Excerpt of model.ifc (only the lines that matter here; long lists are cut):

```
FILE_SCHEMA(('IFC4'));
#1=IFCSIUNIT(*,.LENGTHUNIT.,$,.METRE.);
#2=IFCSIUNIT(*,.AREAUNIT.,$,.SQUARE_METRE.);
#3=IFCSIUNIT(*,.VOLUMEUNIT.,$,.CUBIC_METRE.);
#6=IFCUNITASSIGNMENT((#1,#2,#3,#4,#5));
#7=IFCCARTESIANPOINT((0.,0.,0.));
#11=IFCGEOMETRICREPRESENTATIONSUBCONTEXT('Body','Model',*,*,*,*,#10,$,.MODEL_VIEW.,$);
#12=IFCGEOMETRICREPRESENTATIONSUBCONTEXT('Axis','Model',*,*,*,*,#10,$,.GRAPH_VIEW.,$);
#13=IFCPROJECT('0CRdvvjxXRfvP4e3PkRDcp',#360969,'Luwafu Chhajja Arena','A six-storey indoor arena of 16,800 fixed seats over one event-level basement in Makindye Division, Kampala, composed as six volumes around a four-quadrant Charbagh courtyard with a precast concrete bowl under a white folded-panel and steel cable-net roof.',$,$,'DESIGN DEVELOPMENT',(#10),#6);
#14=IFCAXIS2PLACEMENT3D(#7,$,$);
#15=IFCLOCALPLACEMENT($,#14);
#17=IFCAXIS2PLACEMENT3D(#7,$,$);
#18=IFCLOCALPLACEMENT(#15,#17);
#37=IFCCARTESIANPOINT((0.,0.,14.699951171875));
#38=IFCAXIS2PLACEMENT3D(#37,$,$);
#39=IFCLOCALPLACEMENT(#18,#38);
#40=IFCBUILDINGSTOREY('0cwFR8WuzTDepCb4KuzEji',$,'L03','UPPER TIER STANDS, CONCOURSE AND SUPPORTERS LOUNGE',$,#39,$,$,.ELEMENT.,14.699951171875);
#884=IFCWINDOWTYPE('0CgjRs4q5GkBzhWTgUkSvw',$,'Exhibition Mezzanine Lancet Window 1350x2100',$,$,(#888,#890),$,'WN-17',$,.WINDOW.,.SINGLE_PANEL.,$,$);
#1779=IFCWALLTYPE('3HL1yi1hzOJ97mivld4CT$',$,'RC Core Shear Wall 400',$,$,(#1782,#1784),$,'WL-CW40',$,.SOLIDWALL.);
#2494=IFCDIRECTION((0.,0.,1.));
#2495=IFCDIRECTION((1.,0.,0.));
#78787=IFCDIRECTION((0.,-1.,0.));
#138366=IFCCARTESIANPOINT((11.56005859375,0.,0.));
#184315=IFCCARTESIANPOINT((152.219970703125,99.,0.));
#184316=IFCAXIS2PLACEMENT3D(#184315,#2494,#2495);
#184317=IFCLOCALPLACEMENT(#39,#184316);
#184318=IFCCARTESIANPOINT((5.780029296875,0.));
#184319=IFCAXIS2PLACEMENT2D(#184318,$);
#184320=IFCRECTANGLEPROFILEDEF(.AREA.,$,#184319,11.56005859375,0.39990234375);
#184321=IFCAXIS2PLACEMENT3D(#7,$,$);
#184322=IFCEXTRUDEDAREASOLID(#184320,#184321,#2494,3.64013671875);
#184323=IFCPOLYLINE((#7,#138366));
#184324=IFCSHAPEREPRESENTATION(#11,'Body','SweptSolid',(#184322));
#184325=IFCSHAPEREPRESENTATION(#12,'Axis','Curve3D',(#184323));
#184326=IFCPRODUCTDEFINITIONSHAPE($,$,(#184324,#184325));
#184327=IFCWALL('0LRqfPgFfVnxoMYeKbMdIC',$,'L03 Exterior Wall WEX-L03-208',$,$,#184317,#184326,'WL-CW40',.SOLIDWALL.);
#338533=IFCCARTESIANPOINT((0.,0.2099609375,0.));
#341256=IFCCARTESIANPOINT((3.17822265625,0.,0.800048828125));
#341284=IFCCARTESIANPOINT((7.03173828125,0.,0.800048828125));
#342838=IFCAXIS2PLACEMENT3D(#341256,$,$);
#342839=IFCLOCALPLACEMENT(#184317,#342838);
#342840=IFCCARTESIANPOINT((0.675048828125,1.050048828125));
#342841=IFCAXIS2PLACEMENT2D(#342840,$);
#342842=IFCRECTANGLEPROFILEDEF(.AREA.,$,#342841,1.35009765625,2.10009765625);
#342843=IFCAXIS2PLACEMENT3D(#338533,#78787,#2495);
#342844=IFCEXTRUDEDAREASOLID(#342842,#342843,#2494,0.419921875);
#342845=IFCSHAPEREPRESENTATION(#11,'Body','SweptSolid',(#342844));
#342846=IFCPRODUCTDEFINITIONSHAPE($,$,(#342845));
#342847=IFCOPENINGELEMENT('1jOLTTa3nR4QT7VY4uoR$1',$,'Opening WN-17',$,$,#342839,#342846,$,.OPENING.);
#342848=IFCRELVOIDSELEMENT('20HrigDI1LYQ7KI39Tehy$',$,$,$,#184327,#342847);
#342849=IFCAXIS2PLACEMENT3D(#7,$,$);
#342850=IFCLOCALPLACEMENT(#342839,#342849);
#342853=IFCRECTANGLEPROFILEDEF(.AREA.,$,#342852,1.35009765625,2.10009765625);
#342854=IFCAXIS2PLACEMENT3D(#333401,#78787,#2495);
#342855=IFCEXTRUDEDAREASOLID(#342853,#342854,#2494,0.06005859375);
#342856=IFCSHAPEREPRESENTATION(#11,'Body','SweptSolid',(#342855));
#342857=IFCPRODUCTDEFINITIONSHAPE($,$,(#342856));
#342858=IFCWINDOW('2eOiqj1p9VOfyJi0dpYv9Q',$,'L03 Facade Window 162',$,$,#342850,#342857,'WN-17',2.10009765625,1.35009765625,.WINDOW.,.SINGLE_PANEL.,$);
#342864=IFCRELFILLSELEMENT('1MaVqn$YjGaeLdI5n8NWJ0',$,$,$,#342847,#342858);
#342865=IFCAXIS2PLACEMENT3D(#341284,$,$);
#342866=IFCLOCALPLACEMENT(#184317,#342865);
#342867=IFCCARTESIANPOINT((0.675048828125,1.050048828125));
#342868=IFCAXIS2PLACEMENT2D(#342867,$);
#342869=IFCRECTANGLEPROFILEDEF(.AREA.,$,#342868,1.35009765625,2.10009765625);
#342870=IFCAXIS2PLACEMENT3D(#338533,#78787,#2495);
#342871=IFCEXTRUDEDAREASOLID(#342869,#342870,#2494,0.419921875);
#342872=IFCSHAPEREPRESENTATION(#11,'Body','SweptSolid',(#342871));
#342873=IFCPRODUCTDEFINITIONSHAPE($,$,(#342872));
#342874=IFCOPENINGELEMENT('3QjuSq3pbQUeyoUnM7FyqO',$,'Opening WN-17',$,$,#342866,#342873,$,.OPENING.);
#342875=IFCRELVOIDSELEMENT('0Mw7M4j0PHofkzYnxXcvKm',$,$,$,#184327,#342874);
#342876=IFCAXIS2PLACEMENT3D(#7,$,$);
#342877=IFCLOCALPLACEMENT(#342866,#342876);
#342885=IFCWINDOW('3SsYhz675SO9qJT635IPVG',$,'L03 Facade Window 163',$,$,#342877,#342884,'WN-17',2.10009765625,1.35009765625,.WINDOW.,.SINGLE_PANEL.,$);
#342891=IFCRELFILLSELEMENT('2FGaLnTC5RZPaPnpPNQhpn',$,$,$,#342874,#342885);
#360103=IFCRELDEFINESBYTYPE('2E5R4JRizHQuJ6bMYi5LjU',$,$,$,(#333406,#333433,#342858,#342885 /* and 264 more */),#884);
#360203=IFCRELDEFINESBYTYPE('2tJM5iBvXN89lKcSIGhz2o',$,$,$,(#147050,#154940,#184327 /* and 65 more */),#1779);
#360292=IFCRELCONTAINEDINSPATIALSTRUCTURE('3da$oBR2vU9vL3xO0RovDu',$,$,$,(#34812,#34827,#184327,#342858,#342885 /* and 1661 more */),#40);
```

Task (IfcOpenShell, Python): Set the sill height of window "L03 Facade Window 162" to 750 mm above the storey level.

```python
import numpy as np
import ifcopenshell
import ifcopenshell.api.geometry
import ifcopenshell.geom
import ifcopenshell.util.element
import ifcopenshell.util.placement
import ifcopenshell.util.shape
import ifcopenshell.util.unit

model = ifcopenshell.open("model.ifc")
unit_scale = ifcopenshell.util.unit.calculate_unit_scale(model)

window = model.by_guid("2eOiqj1p9VOfyJi0dpYv9Q")
opening = window.FillsVoids[0].RelatingOpeningElement
storey = ifcopenshell.util.element.get_container(window, ifc_class="IfcBuildingStorey")
level = ifcopenshell.util.placement.get_local_placement(storey.ObjectPlacement)[2, 3]

# The opening's origin need not be at the sill, so measure its lowest point.
shape = ifcopenshell.geom.create_shape(ifcopenshell.geom.settings(), opening)
bottom = ifcopenshell.util.shape.get_shape_bottom_elevation(shape, shape.geometry) / unit_scale
dz = level + 0.75 / unit_scale - bottom

shift = np.array([0.0, 0.0, dz])
# The window is placed relative to its opening, so it follows when the opening moves.
matrix = ifcopenshell.util.placement.get_local_placement(opening.ObjectPlacement)
matrix[:3, 3] += shift
ifcopenshell.api.geometry.edit_object_placement(
    model, product=opening, matrix=matrix, is_si=False, should_transform_children=True
)

print(f"moved by {dz * unit_scale:+.3f} m")

model.write("model_rev.ifc")
```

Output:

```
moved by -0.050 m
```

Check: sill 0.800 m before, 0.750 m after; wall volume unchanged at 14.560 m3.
